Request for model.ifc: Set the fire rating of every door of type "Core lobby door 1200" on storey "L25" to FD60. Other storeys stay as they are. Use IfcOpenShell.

First a look at what the model holds.

```python
import ifcopenshell
import ifcopenshell.util.element

model = ifcopenshell.open("model.ifc")
print(model.schema)
storey = next(s for s in model.by_type("IfcBuildingStorey") if s.Name == "L25")
doors = [e for e in ifcopenshell.util.element.get_decomposition(storey) if e.is_a("IfcDoor")]
seen = {}
for e in doors:
    element_type = ifcopenshell.util.element.get_type(e)
    key = (element_type.Name if element_type != e and element_type else None, ifcopenshell.util.element.get_pset(e, "Pset_DoorCommon", "FireRating"))
    seen[key] = seen.get(key, 0) + 1
for (name, value), count in sorted(seen.items(), key=str):
    print(count, "x", name, "|", value)
```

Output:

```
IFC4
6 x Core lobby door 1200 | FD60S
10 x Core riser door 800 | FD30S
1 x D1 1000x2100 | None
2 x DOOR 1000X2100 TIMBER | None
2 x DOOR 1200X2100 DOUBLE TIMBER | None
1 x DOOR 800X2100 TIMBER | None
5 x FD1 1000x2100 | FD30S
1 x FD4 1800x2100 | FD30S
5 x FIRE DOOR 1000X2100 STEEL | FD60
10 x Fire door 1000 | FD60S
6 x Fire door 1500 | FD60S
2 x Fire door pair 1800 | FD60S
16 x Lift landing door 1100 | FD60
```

```python
import ifcopenshell
import ifcopenshell.api.pset
import ifcopenshell.util.element

model = ifcopenshell.open("model.ifc")

storey = next(s for s in model.by_type("IfcBuildingStorey") if s.Name == "L25")
doors = [e for e in ifcopenshell.util.element.get_decomposition(storey) if e.is_a("IfcDoor")]

count = 0
for e in doors:
    element_type = ifcopenshell.util.element.get_type(e)
    if element_type in (None, e) or element_type.Name != "Core lobby door 1200":
        continue
    # add_pset returns the element's existing set when there is one.
    pset = ifcopenshell.api.pset.add_pset(model, product=e, name="Pset_DoorCommon")
    ifcopenshell.api.pset.edit_pset(model, pset=pset, properties={"FireRating": "FD60"})
    count += 1

print(count, "doors updated")

model.write("model_rev.ifc")
```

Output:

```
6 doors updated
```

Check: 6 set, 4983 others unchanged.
